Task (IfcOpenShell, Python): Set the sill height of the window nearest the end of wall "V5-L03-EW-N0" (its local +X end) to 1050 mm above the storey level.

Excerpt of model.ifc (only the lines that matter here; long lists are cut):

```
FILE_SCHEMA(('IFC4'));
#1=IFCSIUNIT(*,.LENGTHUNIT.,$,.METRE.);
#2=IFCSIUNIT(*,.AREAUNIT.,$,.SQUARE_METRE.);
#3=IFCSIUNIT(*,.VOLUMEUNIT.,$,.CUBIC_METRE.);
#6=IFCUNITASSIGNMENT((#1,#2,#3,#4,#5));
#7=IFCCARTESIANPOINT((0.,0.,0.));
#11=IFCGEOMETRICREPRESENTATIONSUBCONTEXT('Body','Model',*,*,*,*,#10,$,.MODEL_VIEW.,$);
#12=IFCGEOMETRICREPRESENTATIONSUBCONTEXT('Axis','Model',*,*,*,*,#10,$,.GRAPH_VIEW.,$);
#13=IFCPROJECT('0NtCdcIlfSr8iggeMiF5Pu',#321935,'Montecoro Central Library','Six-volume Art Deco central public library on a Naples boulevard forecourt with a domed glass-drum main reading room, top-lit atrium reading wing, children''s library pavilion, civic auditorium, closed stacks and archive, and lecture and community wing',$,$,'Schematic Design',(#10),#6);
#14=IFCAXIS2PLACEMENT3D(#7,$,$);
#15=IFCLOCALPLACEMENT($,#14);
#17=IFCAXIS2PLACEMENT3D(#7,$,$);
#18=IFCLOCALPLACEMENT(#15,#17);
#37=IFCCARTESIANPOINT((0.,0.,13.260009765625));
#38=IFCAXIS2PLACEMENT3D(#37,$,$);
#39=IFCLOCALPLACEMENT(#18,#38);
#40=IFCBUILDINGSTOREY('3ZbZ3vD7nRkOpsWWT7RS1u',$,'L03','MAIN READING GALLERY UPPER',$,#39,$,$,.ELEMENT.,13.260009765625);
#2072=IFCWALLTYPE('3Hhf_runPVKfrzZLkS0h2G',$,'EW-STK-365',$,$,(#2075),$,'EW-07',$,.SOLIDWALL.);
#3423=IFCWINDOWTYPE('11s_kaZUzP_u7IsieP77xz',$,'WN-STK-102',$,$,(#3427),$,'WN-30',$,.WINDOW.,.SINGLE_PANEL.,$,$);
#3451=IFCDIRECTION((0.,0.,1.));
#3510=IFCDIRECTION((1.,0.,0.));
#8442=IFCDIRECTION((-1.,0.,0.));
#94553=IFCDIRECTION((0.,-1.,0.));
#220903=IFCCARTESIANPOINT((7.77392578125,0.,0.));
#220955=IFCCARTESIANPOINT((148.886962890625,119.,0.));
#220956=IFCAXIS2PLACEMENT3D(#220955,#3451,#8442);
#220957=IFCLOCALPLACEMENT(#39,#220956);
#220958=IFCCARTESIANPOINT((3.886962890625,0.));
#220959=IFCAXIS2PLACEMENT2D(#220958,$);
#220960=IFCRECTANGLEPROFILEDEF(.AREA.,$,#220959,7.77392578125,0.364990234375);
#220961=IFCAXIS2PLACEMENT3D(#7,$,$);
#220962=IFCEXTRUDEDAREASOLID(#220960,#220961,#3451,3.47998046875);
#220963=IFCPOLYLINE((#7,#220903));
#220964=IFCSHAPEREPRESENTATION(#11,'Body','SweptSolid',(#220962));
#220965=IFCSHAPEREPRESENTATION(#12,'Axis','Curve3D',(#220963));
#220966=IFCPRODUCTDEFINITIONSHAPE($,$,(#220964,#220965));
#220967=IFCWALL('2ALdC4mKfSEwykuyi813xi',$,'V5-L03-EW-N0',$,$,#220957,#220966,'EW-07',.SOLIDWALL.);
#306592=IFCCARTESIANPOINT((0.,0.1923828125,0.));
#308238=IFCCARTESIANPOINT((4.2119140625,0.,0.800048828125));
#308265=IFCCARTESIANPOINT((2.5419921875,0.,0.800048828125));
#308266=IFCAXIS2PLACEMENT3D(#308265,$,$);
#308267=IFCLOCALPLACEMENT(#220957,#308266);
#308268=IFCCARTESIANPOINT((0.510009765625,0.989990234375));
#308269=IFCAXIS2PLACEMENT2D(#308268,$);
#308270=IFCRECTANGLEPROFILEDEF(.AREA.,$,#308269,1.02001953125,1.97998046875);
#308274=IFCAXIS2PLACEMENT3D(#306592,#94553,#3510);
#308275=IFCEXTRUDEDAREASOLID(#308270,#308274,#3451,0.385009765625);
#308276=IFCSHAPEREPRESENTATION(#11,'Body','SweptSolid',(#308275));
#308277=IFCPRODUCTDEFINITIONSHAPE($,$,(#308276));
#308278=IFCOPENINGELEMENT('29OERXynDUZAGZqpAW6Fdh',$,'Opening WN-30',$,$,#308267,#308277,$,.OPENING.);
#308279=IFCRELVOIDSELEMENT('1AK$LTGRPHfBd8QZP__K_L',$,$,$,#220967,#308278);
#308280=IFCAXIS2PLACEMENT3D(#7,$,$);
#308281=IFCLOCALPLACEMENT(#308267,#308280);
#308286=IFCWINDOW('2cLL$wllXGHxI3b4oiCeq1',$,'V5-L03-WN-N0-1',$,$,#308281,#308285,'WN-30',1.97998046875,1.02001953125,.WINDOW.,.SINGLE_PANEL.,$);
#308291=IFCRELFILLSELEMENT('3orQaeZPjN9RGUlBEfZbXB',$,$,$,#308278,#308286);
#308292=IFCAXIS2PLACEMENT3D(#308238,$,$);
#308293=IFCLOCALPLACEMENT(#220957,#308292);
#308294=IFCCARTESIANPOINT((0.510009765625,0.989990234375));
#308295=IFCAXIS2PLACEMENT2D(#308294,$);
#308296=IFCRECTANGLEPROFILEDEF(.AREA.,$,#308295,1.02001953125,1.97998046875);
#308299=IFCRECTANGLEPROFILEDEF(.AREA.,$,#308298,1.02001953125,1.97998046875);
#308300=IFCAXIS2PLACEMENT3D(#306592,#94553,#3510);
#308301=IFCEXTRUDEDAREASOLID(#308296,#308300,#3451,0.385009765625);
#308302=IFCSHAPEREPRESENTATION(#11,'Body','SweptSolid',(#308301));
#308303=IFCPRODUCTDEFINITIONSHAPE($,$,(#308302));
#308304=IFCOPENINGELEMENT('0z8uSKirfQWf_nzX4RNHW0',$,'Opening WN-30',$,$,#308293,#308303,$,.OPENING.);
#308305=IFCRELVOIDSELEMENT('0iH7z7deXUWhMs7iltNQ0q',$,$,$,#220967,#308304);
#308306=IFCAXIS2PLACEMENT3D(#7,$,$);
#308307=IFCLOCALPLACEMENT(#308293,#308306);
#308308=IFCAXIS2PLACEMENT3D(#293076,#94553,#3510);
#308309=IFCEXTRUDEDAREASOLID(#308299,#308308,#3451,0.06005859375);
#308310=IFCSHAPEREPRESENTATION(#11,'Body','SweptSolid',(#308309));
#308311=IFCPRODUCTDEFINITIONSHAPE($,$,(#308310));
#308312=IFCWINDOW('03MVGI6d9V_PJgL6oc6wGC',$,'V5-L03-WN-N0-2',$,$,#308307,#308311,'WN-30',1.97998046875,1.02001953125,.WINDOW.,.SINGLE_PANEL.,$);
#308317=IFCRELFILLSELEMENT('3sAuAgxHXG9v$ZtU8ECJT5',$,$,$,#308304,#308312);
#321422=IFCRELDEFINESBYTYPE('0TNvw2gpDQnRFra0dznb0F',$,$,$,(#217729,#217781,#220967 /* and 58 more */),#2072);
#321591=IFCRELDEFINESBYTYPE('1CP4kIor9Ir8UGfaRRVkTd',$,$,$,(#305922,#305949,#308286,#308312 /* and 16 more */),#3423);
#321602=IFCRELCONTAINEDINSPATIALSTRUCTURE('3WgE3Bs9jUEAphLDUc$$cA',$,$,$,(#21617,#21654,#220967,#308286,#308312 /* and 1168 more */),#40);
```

```python
import numpy as np
import ifcopenshell
import ifcopenshell.api.geometry
import ifcopenshell.geom
import ifcopenshell.util.element
import ifcopenshell.util.placement
import ifcopenshell.util.shape
import ifcopenshell.util.unit

model = ifcopenshell.open("model.ifc")
unit_scale = ifcopenshell.util.unit.calculate_unit_scale(model)

window = model.by_id(308312)
opening = window.FillsVoids[0].RelatingOpeningElement
storey = ifcopenshell.util.element.get_container(window, ifc_class="IfcBuildingStorey")
level = ifcopenshell.util.placement.get_local_placement(storey.ObjectPlacement)[2, 3]

# The opening's origin need not be at the sill, so measure its lowest point.
shape = ifcopenshell.geom.create_shape(ifcopenshell.geom.settings(), opening)
bottom = ifcopenshell.util.shape.get_shape_bottom_elevation(shape, shape.geometry) / unit_scale
dz = level + 1.05 / unit_scale - bottom

shift = np.array([0.0, 0.0, dz])
# The window is placed relative to its opening, so it follows when the opening moves.
matrix = ifcopenshell.util.placement.get_local_placement(opening.ObjectPlacement)
matrix[:3, 3] += shift
ifcopenshell.api.geometry.edit_object_placement(
    model, product=opening, matrix=matrix, is_si=False, should_transform_children=True
)

print(f"moved by {dz * unit_scale:+.3f} m")

model.write("model_edited.ifc")
```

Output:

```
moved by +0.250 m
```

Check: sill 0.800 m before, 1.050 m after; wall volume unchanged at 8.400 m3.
